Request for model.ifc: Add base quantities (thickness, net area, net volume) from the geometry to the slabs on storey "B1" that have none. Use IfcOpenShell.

First a look at what the model holds.

```python
import ifcopenshell
import ifcopenshell.util.element
import ifcopenshell.util.unit

model = ifcopenshell.open("model.ifc")
print(model.schema)
for unit_type in ("LENGTHUNIT", "AREAUNIT", "VOLUMEUNIT"):
    print(unit_type, ifcopenshell.util.unit.calculate_unit_scale(model, unit_type))
storey = next(s for s in model.by_type("IfcBuildingStorey") if s.Name == "B1")
slabs = [e for e in ifcopenshell.util.element.get_decomposition(storey) if e.is_a("IfcSlab")]
for e in sorted(slabs, key=lambda e: e.id()):
    print(e.id(), e.is_a(), e.Name, list(ifcopenshell.util.element.get_psets(e, qtos_only=True)), sep=" | ")
```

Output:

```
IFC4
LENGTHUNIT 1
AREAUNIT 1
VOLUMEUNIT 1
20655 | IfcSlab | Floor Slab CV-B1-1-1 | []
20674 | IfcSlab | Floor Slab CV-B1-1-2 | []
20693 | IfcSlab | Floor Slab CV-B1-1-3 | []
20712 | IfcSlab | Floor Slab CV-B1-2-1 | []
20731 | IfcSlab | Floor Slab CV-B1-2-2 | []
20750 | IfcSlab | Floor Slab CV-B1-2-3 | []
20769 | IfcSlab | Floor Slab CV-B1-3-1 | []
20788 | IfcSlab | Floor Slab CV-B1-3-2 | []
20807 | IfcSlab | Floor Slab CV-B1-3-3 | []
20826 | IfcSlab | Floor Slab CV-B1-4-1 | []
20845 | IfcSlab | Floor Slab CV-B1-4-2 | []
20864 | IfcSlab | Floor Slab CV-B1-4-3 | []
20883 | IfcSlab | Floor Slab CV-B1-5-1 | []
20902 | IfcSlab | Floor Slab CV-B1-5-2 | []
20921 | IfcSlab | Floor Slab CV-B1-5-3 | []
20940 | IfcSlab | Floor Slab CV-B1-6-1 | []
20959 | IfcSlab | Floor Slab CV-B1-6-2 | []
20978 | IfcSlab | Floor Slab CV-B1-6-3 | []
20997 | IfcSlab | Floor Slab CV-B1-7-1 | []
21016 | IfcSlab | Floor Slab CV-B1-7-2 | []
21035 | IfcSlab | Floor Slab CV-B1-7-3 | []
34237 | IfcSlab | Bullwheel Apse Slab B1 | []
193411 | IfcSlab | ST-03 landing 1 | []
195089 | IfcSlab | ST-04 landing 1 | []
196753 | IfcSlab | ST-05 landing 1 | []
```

```python
import ifcopenshell
import ifcopenshell.api.pset
import ifcopenshell.geom
import ifcopenshell.util.element
import ifcopenshell.util.shape
import ifcopenshell.util.unit

model = ifcopenshell.open("model.ifc")
unit_scale = ifcopenshell.util.unit.calculate_unit_scale(model)
area_scale = ifcopenshell.util.unit.calculate_unit_scale(model, "AREAUNIT")
volume_scale = ifcopenshell.util.unit.calculate_unit_scale(model, "VOLUMEUNIT")
settings = ifcopenshell.geom.settings()

storey = next(s for s in model.by_type("IfcBuildingStorey") if s.Name == "B1")
slabs = [e for e in ifcopenshell.util.element.get_decomposition(storey) if e.is_a("IfcSlab")]

for e in sorted(slabs, key=lambda e: e.id()):
    if ifcopenshell.util.element.get_psets(e, qtos_only=True, should_inherit=False):
        continue
    # Geometry comes back in metres, in the element's own axes.
    shape = ifcopenshell.geom.create_shape(settings, e)
    values = {
        "Width": ifcopenshell.util.shape.get_z(shape.geometry) / unit_scale,
        "NetArea": ifcopenshell.util.shape.get_footprint_area(shape.geometry) / area_scale,
        "NetVolume": ifcopenshell.util.shape.get_volume(shape.geometry) / volume_scale,
    }
    qto = ifcopenshell.api.pset.add_qto(model, product=e, name="Qto_SlabBaseQuantities")
    ifcopenshell.api.pset.edit_qto(model, qto=qto, properties=values)
    print(e.id(), {k: round(v, 3) for k, v in values.items()})

model.write("model_updated.ifc")
```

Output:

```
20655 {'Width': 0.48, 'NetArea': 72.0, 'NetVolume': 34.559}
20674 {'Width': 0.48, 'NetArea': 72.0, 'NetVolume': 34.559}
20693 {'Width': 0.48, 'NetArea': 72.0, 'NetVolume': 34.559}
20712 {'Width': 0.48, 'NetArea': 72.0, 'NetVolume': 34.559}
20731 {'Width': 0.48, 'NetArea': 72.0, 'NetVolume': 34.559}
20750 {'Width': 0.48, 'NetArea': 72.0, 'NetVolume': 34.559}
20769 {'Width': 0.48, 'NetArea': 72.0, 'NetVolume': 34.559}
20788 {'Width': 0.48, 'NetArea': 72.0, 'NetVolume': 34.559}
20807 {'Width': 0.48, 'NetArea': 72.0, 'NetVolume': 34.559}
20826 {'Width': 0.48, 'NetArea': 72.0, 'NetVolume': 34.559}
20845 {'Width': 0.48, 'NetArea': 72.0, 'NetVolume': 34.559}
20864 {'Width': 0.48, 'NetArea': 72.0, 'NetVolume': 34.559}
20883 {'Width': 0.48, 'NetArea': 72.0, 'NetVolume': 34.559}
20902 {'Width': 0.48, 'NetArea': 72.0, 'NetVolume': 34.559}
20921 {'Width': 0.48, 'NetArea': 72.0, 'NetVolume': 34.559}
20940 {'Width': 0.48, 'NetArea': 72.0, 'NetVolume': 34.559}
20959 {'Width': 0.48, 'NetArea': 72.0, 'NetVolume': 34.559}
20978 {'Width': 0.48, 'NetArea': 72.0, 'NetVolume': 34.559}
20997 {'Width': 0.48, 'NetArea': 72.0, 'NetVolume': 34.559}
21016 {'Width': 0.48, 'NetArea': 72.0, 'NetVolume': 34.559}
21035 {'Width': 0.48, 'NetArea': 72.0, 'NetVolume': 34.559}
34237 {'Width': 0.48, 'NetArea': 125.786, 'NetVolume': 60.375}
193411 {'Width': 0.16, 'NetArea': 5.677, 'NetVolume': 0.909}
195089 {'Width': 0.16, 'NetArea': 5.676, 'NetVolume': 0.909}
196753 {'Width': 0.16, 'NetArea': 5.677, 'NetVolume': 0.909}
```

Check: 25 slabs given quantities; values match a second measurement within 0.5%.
